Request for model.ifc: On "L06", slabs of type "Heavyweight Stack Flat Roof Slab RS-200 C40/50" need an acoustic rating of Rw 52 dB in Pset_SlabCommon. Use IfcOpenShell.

First a look at what the model holds.

```python
import ifcopenshell
import ifcopenshell.util.element

model = ifcopenshell.open("model.ifc")
print(model.schema)
storey = next(s for s in model.by_type("IfcBuildingStorey") if s.Name == "L06")
slabs = [e for e in ifcopenshell.util.element.get_decomposition(storey) if e.is_a("IfcSlab")]
seen = {}
for e in slabs:
    element_type = ifcopenshell.util.element.get_type(e)
    key = (element_type.Name if element_type != e and element_type else None, ifcopenshell.util.element.get_pset(e, "Pset_SlabCommon", "AcousticRating"))
    seen[key] = seen.get(key, 0) + 1
for (name, value), count in sorted(seen.items(), key=str):
    print(count, "x", name, "|", value)
```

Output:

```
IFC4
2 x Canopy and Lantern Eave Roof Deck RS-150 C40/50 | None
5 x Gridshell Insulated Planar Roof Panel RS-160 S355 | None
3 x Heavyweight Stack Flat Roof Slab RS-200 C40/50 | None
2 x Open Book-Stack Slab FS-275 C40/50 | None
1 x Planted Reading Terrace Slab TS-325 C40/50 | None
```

```python
import ifcopenshell
import ifcopenshell.api.pset
import ifcopenshell.util.element

model = ifcopenshell.open("model.ifc")

storey = next(s for s in model.by_type("IfcBuildingStorey") if s.Name == "L06")
slabs = [e for e in ifcopenshell.util.element.get_decomposition(storey) if e.is_a("IfcSlab")]

count = 0
for e in slabs:
    element_type = ifcopenshell.util.element.get_type(e)
    if element_type in (None, e) or element_type.Name != "Heavyweight Stack Flat Roof Slab RS-200 C40/50":
        continue
    # add_pset returns the element's existing set when there is one.
    pset = ifcopenshell.api.pset.add_pset(model, product=e, name="Pset_SlabCommon")
    ifcopenshell.api.pset.edit_pset(model, pset=pset, properties={"AcousticRating": "Rw 52 dB"})
    count += 1

print(count, "slabs updated")

model.write("model_updated.ifc")
```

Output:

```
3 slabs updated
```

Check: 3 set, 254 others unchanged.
